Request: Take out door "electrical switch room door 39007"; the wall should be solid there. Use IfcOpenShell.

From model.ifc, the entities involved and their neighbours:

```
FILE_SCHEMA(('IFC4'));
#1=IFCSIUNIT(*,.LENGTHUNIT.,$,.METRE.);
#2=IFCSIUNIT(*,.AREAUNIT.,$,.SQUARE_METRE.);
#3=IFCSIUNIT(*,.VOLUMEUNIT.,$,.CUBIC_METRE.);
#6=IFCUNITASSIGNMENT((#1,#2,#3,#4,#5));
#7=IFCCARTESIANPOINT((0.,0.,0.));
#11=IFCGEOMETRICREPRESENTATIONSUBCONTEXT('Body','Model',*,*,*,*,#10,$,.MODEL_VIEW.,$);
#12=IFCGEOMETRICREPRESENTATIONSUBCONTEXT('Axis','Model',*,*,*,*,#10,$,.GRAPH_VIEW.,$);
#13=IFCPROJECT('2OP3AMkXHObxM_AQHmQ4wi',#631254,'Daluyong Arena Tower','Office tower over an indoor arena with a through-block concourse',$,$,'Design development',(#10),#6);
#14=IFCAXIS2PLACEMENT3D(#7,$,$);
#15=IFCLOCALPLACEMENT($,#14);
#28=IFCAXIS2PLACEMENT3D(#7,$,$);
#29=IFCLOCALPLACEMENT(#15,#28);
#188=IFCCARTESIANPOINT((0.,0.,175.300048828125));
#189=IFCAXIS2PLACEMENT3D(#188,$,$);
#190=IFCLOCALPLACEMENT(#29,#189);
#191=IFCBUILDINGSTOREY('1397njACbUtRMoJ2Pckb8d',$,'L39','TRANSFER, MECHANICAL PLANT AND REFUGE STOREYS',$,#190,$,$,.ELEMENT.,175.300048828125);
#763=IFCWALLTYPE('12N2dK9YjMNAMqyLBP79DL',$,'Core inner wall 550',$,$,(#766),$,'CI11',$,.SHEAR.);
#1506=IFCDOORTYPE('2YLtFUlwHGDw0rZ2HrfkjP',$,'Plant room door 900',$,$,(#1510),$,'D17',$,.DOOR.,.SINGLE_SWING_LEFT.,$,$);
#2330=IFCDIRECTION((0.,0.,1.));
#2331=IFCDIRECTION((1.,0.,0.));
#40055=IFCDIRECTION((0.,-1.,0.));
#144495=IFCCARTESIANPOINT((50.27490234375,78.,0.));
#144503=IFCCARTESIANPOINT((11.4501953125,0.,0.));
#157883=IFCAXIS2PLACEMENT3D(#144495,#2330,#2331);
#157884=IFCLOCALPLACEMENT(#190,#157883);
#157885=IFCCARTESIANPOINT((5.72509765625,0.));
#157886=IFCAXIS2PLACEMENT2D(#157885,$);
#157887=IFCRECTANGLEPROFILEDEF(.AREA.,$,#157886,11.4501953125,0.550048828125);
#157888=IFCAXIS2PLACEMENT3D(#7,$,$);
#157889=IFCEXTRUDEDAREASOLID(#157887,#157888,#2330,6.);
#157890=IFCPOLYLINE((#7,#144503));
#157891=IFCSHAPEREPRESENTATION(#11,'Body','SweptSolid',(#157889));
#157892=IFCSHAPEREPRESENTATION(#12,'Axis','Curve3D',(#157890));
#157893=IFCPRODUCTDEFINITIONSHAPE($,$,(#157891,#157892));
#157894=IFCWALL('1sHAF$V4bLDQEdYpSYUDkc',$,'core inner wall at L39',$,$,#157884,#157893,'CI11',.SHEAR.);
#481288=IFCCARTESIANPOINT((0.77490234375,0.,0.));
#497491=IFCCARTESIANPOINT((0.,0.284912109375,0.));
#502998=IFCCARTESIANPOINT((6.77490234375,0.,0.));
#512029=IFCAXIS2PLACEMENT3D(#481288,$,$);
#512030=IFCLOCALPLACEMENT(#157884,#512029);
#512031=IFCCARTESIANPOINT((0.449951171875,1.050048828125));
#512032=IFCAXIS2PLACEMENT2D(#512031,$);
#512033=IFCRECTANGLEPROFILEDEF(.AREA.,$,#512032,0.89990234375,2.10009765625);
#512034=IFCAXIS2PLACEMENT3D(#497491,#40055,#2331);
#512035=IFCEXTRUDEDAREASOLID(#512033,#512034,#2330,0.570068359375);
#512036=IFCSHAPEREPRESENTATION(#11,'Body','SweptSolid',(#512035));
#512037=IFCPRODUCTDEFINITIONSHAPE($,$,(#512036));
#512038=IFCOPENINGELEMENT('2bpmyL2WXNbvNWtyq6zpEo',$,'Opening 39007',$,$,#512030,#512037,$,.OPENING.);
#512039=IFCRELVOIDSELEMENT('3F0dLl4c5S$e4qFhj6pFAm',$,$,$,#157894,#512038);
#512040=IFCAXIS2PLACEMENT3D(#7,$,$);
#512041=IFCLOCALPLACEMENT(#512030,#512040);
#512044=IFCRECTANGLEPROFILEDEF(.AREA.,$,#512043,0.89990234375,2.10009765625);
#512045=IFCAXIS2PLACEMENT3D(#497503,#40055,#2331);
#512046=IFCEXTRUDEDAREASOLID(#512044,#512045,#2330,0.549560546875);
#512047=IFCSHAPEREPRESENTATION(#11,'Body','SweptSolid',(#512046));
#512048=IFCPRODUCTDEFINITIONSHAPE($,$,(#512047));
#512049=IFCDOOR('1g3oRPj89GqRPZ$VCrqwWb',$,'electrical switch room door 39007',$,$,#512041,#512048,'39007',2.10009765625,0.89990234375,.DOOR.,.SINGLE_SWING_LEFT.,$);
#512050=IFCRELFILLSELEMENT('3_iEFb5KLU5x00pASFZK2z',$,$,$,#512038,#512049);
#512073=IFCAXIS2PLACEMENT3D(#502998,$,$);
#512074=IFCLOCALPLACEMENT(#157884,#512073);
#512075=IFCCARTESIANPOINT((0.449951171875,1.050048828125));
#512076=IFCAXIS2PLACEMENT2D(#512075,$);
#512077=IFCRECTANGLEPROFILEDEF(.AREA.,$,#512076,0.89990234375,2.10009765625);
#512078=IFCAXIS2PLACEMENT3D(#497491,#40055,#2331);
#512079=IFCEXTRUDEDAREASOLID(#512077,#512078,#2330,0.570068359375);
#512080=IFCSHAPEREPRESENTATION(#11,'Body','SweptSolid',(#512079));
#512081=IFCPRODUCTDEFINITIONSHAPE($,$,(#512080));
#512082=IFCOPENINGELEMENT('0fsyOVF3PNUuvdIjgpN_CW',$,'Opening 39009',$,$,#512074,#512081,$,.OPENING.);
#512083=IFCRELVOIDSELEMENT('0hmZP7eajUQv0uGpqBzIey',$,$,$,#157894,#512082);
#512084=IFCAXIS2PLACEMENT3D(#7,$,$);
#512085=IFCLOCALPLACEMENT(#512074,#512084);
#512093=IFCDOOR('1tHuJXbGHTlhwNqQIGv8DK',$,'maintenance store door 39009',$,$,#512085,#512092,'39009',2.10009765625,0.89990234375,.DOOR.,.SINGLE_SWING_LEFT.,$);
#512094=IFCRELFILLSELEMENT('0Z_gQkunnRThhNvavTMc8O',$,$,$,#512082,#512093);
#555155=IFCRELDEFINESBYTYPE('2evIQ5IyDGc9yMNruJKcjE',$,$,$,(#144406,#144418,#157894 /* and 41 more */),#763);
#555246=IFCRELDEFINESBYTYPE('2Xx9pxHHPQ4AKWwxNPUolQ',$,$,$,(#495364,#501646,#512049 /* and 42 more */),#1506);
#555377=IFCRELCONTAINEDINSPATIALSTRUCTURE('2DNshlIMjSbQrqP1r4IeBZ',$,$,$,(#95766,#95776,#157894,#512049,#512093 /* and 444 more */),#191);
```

```python
import ifcopenshell
import ifcopenshell.api.feature
import ifcopenshell.api.root
import ifcopenshell.geom
import ifcopenshell.util.shape

model = ifcopenshell.open("model.ifc")
settings = ifcopenshell.geom.settings()


def volume(element):
    """Net volume in cubic metres, openings subtracted."""
    shape = ifcopenshell.geom.create_shape(settings, element)
    return ifcopenshell.util.shape.get_volume(shape.geometry)


door = model.by_guid("1g3oRPj89GqRPZ$VCrqwWb")
opening = door.FillsVoids[0].RelatingOpeningElement
wall = opening.VoidsElements[0].RelatingBuildingElement
before = volume(wall)

ifcopenshell.api.root.remove_product(model, product=door)
ifcopenshell.api.feature.remove_feature(model, feature=opening)

after = volume(wall)

print(f"wall volume {before:.3f} -> {after:.3f} m3")

model.write("model_rev.ifc")
```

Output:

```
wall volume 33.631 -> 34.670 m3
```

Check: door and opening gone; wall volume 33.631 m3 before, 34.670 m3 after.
